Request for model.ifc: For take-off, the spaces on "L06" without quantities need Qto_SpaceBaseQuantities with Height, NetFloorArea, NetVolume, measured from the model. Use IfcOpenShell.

First a look at what the model holds.

```python
import ifcopenshell
import ifcopenshell.util.element
import ifcopenshell.util.unit

model = ifcopenshell.open("model.ifc")
print(model.schema)
for unit_type in ("LENGTHUNIT", "AREAUNIT", "VOLUMEUNIT"):
    print(unit_type, ifcopenshell.util.unit.calculate_unit_scale(model, unit_type))
storey = next(s for s in model.by_type("IfcBuildingStorey") if s.Name == "L06")
spaces = [e for e in ifcopenshell.util.element.get_decomposition(storey) if e.is_a("IfcSpace")]
for e in sorted(spaces, key=lambda e: e.id()):
    print(e.id(), e.is_a(), e.Name, list(ifcopenshell.util.element.get_psets(e, qtos_only=True)), sep=" | ")
```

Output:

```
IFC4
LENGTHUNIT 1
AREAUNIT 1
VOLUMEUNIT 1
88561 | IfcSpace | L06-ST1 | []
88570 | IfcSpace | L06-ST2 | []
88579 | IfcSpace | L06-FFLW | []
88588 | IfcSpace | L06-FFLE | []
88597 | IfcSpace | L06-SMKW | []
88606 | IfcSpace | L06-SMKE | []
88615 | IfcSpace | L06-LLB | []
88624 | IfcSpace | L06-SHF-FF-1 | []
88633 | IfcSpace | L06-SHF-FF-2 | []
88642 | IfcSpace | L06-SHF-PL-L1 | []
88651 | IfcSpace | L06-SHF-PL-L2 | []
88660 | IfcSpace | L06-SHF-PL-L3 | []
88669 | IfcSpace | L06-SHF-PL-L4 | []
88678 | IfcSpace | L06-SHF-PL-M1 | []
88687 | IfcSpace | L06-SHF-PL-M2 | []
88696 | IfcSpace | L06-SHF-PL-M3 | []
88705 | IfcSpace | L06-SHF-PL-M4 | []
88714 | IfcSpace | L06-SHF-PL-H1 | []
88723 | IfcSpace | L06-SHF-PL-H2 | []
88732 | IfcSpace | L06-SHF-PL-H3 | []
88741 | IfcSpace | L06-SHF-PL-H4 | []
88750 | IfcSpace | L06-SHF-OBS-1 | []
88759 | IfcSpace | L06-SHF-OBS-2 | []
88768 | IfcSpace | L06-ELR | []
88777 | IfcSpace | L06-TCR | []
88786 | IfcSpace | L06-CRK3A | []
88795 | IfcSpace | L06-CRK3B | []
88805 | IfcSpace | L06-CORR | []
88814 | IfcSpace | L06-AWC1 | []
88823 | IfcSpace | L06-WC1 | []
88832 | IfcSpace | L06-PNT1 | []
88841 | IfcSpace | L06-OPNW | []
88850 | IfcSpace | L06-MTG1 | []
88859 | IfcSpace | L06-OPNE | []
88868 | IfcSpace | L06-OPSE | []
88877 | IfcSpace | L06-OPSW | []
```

```python
import ifcopenshell
import ifcopenshell.api.pset
import ifcopenshell.geom
import ifcopenshell.util.element
import ifcopenshell.util.shape
import ifcopenshell.util.unit

model = ifcopenshell.open("model.ifc")
unit_scale = ifcopenshell.util.unit.calculate_unit_scale(model)
area_scale = ifcopenshell.util.unit.calculate_unit_scale(model, "AREAUNIT")
volume_scale = ifcopenshell.util.unit.calculate_unit_scale(model, "VOLUMEUNIT")
settings = ifcopenshell.geom.settings()

storey = next(s for s in model.by_type("IfcBuildingStorey") if s.Name == "L06")
spaces = [e for e in ifcopenshell.util.element.get_decomposition(storey) if e.is_a("IfcSpace")]

for e in sorted(spaces, key=lambda e: e.id()):
    if ifcopenshell.util.element.get_psets(e, qtos_only=True, should_inherit=False):
        continue
    # Geometry comes back in metres, in the element's own axes.
    shape = ifcopenshell.geom.create_shape(settings, e)
    values = {
        "Height": ifcopenshell.util.shape.get_z(shape.geometry) / unit_scale,
        "NetFloorArea": ifcopenshell.util.shape.get_footprint_area(shape.geometry) / area_scale,
        "NetVolume": ifcopenshell.util.shape.get_volume(shape.geometry) / volume_scale,
    }
    qto = ifcopenshell.api.pset.add_qto(model, product=e, name="Qto_SpaceBaseQuantities")
    ifcopenshell.api.pset.edit_qto(model, qto=qto, properties=values)
    print(e.id(), {k: round(v, 3) for k, v in values.items()})

model.write("model_rev.ifc")
```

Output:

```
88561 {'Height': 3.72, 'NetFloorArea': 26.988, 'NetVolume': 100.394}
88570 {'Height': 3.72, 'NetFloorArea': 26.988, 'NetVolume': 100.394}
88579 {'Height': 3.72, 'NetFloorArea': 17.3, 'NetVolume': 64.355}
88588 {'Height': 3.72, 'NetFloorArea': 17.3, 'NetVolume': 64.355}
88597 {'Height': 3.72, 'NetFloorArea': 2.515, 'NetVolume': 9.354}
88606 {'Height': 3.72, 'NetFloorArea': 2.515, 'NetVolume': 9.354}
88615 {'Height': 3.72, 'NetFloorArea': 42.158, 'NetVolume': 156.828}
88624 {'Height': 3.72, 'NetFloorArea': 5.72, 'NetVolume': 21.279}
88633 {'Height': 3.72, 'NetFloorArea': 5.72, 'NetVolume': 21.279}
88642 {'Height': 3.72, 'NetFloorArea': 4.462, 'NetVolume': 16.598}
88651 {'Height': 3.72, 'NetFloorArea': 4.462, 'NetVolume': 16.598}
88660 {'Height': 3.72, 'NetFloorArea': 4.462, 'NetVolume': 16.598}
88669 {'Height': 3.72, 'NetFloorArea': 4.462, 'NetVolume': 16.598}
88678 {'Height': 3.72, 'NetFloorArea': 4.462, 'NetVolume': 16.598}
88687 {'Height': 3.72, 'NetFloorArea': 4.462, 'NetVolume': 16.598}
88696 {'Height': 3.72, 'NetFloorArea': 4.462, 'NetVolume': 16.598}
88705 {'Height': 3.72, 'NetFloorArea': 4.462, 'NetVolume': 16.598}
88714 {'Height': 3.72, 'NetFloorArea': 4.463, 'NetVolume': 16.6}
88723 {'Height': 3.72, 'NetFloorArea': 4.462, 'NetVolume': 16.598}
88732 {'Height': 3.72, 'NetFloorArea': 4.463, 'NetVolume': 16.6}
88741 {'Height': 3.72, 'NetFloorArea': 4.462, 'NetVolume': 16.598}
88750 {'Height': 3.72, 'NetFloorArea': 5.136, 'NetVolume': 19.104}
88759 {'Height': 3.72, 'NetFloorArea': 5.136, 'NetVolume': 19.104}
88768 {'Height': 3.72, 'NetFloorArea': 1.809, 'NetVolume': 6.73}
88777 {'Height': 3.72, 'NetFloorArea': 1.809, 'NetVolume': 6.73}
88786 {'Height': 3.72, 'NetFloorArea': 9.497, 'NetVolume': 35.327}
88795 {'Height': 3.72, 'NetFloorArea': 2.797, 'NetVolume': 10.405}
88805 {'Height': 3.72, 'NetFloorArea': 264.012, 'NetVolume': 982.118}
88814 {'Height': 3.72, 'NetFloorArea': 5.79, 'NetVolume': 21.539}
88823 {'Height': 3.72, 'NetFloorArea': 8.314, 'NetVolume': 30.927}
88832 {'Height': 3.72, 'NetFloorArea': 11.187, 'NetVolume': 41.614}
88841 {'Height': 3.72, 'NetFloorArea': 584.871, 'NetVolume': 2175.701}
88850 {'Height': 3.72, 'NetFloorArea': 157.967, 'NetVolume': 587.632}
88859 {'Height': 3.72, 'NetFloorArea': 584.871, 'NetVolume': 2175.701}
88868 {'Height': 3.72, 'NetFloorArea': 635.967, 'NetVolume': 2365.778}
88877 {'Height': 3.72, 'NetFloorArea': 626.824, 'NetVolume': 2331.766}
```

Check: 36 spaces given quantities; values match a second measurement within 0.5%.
